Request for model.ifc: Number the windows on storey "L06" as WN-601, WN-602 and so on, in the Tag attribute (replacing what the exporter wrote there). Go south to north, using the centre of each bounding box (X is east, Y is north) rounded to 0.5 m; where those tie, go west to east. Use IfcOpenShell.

First a look at what the model holds.

```python
import ifcopenshell
import ifcopenshell.util.element
import ifcopenshell.util.placement

model = ifcopenshell.open("model.ifc")
print(model.schema)
storey = next(s for s in model.by_type("IfcBuildingStorey") if s.Name == "L06")
windows = [e for e in ifcopenshell.util.element.get_decomposition(storey) if e.is_a("IfcWindow")]
for e in sorted(windows, key=lambda e: e.id()):
    origin = ifcopenshell.util.placement.get_local_placement(e.ObjectPlacement)[:3, 3]
    print(e.id(), e.Tag, e.Name, origin.round(2) + 0.0, sep=" | ")
```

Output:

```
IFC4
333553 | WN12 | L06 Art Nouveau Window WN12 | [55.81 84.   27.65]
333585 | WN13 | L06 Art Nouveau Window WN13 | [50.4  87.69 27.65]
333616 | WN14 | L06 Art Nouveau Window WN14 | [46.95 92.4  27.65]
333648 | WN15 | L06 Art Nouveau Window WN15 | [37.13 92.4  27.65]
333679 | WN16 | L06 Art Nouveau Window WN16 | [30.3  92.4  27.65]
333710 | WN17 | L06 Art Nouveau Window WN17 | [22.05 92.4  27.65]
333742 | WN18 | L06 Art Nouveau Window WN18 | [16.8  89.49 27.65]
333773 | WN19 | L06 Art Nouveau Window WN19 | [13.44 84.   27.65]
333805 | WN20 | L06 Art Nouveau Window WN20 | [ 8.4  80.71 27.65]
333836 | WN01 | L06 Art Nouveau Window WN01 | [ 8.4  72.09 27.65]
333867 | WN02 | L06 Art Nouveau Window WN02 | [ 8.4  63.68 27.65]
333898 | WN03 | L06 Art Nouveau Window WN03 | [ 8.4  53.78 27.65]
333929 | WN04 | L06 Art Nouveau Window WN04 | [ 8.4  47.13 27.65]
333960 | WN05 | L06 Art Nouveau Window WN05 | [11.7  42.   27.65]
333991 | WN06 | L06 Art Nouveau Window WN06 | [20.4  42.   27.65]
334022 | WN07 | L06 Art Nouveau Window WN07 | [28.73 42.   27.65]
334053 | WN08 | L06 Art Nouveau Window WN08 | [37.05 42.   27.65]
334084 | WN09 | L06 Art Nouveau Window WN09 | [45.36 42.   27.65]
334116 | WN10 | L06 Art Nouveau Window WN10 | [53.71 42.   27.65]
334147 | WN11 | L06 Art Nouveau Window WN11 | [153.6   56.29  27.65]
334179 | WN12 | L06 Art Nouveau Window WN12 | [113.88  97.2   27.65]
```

```python
import ifcopenshell
import ifcopenshell.geom
import ifcopenshell.util.element
import ifcopenshell.util.shape

model = ifcopenshell.open("model.ifc")
settings = ifcopenshell.geom.settings()
settings.set("use-world-coords", True)


def centre(element):
    shape = ifcopenshell.geom.create_shape(settings, element)
    return ifcopenshell.util.shape.get_bbox_centroid(shape.geometry)


storey = next(s for s in model.by_type("IfcBuildingStorey") if s.Name == "L06")
windows = [e for e in ifcopenshell.util.element.get_decomposition(storey) if e.is_a("IfcWindow")]

# Insertion points can sit at a corner or the storey origin, so sort by the geometry (in metres).
centres = {e: centre(e) for e in windows}
windows.sort(key=lambda e: (round(centres[e][1] / 0.5), centres[e][0]))

for i, e in enumerate(windows, start=1):
    number = f"WN-6{i:02d}"
    e.Tag = number
    print(e.id(), number)

model.write("model_updated.ifc")
```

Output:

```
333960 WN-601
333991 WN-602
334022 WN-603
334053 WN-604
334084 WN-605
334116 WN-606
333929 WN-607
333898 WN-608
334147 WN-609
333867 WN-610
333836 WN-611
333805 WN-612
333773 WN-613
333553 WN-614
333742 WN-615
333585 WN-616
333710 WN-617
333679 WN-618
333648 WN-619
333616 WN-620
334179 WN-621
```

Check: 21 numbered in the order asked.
